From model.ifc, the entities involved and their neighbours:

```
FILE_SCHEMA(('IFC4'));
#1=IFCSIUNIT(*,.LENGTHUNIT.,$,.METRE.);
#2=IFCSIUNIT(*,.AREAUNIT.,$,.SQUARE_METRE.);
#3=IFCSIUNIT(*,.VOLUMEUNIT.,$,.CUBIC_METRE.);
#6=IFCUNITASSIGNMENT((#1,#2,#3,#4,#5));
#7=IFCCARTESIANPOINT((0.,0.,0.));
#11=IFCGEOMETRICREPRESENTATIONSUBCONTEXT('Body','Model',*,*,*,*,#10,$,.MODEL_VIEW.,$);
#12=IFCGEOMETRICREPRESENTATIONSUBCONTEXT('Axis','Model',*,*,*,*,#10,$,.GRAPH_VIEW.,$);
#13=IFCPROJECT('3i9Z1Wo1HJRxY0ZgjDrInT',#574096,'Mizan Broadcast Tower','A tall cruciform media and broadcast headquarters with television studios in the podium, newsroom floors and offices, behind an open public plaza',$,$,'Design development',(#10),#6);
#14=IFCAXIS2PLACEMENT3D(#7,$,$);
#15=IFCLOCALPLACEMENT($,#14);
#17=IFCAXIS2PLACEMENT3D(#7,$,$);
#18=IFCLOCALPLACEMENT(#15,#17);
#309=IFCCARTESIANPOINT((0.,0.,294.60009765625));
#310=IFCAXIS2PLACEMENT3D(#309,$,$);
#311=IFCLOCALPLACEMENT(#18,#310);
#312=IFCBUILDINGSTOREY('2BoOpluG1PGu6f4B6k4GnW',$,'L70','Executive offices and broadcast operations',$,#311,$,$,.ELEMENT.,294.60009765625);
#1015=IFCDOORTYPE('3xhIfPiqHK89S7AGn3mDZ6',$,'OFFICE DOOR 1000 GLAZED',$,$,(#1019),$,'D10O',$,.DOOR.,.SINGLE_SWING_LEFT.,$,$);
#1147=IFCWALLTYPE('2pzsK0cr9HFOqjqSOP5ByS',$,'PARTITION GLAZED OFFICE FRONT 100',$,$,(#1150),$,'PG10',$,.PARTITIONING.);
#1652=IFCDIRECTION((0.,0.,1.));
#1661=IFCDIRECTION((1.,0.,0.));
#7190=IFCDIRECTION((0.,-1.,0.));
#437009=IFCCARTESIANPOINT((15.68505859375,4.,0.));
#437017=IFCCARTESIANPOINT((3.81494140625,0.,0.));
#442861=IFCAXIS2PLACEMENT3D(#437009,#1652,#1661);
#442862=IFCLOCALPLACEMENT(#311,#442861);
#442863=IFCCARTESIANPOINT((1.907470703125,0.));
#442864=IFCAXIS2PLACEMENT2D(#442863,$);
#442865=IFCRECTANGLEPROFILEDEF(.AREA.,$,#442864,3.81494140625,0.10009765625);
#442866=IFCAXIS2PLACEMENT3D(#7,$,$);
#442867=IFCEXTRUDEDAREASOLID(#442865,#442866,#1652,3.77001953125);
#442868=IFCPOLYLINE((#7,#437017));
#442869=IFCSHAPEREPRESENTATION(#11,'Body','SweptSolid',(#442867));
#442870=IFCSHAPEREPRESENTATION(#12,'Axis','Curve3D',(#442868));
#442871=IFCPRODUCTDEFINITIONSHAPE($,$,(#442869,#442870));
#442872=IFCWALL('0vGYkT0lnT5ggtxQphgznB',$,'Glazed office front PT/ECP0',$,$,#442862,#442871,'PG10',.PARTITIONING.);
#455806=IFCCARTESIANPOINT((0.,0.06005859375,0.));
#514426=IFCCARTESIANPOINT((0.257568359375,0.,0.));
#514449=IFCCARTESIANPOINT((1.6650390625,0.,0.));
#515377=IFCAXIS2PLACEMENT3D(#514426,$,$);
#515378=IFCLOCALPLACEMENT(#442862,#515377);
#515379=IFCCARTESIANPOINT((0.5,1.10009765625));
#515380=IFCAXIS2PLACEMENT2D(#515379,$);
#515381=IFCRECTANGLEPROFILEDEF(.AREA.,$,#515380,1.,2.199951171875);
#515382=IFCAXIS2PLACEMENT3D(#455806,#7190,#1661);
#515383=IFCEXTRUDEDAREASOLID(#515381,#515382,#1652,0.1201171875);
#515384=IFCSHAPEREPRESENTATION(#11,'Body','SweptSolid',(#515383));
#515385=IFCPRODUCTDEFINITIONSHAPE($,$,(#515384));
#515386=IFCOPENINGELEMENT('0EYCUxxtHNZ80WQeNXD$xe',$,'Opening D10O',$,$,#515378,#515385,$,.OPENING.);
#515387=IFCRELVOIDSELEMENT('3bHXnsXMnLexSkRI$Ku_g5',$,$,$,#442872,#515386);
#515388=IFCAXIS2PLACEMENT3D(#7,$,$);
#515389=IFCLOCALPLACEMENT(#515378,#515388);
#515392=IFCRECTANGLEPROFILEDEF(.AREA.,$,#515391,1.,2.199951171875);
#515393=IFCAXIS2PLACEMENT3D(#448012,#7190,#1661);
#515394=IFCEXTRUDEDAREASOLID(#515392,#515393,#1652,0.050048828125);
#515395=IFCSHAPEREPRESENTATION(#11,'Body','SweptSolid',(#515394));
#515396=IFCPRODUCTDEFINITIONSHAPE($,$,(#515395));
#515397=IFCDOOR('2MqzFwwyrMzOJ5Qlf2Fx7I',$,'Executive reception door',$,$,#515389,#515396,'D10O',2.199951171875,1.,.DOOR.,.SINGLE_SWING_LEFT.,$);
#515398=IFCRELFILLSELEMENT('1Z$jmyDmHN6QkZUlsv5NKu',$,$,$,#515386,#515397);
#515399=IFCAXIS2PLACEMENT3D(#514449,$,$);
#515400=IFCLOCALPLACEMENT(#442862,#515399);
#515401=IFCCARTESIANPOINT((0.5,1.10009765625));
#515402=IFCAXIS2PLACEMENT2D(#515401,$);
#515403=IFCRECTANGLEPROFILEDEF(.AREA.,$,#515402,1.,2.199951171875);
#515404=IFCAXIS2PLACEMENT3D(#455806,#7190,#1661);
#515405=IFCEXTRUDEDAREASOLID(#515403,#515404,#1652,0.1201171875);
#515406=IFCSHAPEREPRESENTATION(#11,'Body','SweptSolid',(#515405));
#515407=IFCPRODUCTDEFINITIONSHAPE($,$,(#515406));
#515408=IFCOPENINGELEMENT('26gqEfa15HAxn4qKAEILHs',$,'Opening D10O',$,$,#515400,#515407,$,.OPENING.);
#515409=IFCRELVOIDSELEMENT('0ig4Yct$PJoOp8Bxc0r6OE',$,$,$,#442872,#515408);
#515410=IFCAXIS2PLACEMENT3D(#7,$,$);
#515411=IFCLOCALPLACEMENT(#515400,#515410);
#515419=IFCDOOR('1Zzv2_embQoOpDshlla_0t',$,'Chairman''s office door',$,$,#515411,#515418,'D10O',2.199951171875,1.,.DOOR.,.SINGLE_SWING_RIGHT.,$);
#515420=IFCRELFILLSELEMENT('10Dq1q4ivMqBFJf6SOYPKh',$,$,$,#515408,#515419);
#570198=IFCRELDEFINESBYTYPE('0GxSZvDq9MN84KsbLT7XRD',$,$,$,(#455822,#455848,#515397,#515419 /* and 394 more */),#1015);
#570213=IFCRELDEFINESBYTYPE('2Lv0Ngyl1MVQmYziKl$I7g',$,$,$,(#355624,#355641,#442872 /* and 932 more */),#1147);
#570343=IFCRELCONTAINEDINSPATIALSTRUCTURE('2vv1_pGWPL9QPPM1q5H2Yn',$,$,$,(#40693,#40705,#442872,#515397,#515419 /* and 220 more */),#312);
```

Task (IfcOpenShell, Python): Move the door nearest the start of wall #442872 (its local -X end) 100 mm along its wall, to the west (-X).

```python
import ifcopenshell
import ifcopenshell.api.geometry
import ifcopenshell.util.placement
import ifcopenshell.util.unit

model = ifcopenshell.open("model.ifc")
unit_scale = ifcopenshell.util.unit.calculate_unit_scale(model)

door = model.by_guid("2MqzFwwyrMzOJ5Qlf2Fx7I")
opening = door.FillsVoids[0].RelatingOpeningElement
wall = opening.VoidsElements[0].RelatingBuildingElement

wall_matrix = ifcopenshell.util.placement.get_local_placement(wall.ObjectPlacement)
shift = wall_matrix[:3, 0] * -0.1 / unit_scale
before = ifcopenshell.util.placement.get_local_placement(door.ObjectPlacement)[:3, 3].copy()

# The door is placed relative to its opening, so it follows when the opening moves.
matrix = ifcopenshell.util.placement.get_local_placement(opening.ObjectPlacement)
matrix[:3, 3] += shift
ifcopenshell.api.geometry.edit_object_placement(
    model, product=opening, matrix=matrix, is_si=False, should_transform_children=True
)

after = ifcopenshell.util.placement.get_local_placement(door.ObjectPlacement)[:3, 3]
print("door moved by", (after - before).round(3) + 0.0)

model.write("model_rev.ifc")
```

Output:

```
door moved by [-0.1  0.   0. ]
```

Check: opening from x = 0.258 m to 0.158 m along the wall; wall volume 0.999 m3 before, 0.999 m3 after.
